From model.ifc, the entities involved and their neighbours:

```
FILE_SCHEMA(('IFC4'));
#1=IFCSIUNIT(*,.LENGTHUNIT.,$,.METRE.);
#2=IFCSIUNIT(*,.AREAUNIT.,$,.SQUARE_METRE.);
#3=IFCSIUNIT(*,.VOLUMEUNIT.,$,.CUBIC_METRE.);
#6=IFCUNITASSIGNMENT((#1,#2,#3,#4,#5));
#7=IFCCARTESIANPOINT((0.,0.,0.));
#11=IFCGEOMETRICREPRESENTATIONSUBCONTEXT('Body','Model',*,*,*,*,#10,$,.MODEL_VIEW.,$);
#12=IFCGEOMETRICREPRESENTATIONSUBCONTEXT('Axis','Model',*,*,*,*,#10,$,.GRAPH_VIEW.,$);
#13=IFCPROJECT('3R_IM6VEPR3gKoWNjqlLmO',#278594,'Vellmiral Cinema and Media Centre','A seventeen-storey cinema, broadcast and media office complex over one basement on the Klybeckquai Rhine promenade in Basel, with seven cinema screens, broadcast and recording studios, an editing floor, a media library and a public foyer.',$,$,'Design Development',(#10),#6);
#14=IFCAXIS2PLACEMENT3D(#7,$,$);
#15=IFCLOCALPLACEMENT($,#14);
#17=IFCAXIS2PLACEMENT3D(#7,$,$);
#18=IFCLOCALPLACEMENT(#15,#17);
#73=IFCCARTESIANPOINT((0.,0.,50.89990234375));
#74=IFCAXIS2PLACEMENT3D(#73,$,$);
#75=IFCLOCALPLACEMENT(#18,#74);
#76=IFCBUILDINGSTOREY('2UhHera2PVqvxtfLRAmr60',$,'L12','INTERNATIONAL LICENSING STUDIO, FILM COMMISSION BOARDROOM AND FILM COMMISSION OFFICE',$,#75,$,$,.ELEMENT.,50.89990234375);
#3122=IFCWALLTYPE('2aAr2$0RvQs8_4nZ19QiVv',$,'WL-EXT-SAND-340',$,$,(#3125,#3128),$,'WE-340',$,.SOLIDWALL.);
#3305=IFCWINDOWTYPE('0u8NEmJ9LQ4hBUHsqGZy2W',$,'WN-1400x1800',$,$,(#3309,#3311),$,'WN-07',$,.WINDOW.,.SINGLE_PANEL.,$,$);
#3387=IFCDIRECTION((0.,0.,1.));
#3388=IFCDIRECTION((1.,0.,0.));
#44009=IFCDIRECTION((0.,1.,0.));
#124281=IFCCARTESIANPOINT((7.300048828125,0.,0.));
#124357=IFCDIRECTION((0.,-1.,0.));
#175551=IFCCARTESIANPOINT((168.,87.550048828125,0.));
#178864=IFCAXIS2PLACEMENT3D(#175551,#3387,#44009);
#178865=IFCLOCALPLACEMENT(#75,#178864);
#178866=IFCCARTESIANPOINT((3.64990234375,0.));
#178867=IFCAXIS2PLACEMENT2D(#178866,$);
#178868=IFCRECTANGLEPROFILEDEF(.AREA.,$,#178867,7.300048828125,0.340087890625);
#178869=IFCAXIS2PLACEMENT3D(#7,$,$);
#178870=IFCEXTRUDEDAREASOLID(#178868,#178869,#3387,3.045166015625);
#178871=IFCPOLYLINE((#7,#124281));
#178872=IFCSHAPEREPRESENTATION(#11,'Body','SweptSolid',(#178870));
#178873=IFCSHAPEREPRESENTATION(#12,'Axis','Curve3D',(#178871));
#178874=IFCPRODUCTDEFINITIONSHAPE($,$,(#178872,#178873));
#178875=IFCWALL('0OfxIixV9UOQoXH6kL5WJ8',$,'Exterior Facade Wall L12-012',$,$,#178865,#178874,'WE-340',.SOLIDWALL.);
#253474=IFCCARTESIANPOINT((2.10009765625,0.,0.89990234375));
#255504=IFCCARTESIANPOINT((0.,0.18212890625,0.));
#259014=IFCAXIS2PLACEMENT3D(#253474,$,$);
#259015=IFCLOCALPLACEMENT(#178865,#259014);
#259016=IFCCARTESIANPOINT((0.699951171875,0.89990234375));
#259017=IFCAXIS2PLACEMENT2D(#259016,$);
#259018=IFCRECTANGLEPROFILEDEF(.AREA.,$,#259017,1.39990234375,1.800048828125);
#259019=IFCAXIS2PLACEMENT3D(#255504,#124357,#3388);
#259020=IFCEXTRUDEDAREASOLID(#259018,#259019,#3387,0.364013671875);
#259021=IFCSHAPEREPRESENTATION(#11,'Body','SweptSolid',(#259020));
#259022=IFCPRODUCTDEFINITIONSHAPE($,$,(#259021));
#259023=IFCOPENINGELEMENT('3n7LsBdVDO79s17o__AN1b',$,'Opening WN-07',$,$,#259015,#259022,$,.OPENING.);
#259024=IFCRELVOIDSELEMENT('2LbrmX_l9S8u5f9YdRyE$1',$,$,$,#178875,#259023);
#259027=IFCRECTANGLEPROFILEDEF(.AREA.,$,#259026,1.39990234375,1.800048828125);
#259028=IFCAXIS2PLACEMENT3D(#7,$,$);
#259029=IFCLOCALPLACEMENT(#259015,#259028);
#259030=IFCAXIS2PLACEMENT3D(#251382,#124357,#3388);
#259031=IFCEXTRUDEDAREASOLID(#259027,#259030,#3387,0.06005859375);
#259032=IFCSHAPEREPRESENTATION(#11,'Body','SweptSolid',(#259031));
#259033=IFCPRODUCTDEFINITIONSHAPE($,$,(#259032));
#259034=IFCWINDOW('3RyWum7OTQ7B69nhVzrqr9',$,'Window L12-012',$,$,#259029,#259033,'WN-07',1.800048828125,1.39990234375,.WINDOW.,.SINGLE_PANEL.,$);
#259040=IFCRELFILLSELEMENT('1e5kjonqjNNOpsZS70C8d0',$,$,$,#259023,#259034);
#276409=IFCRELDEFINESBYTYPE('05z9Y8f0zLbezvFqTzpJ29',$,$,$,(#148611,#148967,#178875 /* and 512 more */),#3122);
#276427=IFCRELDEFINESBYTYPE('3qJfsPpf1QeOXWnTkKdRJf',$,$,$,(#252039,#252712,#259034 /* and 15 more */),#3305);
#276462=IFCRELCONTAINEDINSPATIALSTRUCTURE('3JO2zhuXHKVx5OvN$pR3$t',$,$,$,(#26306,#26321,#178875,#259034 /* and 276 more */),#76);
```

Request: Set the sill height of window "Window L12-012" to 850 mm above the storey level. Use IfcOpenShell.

```python
import numpy as np
import ifcopenshell
import ifcopenshell.api.geometry
import ifcopenshell.geom
import ifcopenshell.util.element
import ifcopenshell.util.placement
import ifcopenshell.util.shape
import ifcopenshell.util.unit

model = ifcopenshell.open("model.ifc")
unit_scale = ifcopenshell.util.unit.calculate_unit_scale(model)

window = model.by_guid("3RyWum7OTQ7B69nhVzrqr9")
opening = window.FillsVoids[0].RelatingOpeningElement
storey = ifcopenshell.util.element.get_container(window, ifc_class="IfcBuildingStorey")
level = ifcopenshell.util.placement.get_local_placement(storey.ObjectPlacement)[2, 3]

# The opening's origin need not be at the sill, so measure its lowest point.
shape = ifcopenshell.geom.create_shape(ifcopenshell.geom.settings(), opening)
bottom = ifcopenshell.util.shape.get_shape_bottom_elevation(shape, shape.geometry) / unit_scale
dz = level + 0.85 / unit_scale - bottom

shift = np.array([0.0, 0.0, dz])
# The window is placed relative to its opening, so it follows when the opening moves.
matrix = ifcopenshell.util.placement.get_local_placement(opening.ObjectPlacement)
matrix[:3, 3] += shift
ifcopenshell.api.geometry.edit_object_placement(
    model, product=opening, matrix=matrix, is_si=False, should_transform_children=True
)

print(f"moved by {dz * unit_scale:+.3f} m")

model.write("model_rev.ifc")
```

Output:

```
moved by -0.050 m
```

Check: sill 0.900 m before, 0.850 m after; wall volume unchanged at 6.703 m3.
